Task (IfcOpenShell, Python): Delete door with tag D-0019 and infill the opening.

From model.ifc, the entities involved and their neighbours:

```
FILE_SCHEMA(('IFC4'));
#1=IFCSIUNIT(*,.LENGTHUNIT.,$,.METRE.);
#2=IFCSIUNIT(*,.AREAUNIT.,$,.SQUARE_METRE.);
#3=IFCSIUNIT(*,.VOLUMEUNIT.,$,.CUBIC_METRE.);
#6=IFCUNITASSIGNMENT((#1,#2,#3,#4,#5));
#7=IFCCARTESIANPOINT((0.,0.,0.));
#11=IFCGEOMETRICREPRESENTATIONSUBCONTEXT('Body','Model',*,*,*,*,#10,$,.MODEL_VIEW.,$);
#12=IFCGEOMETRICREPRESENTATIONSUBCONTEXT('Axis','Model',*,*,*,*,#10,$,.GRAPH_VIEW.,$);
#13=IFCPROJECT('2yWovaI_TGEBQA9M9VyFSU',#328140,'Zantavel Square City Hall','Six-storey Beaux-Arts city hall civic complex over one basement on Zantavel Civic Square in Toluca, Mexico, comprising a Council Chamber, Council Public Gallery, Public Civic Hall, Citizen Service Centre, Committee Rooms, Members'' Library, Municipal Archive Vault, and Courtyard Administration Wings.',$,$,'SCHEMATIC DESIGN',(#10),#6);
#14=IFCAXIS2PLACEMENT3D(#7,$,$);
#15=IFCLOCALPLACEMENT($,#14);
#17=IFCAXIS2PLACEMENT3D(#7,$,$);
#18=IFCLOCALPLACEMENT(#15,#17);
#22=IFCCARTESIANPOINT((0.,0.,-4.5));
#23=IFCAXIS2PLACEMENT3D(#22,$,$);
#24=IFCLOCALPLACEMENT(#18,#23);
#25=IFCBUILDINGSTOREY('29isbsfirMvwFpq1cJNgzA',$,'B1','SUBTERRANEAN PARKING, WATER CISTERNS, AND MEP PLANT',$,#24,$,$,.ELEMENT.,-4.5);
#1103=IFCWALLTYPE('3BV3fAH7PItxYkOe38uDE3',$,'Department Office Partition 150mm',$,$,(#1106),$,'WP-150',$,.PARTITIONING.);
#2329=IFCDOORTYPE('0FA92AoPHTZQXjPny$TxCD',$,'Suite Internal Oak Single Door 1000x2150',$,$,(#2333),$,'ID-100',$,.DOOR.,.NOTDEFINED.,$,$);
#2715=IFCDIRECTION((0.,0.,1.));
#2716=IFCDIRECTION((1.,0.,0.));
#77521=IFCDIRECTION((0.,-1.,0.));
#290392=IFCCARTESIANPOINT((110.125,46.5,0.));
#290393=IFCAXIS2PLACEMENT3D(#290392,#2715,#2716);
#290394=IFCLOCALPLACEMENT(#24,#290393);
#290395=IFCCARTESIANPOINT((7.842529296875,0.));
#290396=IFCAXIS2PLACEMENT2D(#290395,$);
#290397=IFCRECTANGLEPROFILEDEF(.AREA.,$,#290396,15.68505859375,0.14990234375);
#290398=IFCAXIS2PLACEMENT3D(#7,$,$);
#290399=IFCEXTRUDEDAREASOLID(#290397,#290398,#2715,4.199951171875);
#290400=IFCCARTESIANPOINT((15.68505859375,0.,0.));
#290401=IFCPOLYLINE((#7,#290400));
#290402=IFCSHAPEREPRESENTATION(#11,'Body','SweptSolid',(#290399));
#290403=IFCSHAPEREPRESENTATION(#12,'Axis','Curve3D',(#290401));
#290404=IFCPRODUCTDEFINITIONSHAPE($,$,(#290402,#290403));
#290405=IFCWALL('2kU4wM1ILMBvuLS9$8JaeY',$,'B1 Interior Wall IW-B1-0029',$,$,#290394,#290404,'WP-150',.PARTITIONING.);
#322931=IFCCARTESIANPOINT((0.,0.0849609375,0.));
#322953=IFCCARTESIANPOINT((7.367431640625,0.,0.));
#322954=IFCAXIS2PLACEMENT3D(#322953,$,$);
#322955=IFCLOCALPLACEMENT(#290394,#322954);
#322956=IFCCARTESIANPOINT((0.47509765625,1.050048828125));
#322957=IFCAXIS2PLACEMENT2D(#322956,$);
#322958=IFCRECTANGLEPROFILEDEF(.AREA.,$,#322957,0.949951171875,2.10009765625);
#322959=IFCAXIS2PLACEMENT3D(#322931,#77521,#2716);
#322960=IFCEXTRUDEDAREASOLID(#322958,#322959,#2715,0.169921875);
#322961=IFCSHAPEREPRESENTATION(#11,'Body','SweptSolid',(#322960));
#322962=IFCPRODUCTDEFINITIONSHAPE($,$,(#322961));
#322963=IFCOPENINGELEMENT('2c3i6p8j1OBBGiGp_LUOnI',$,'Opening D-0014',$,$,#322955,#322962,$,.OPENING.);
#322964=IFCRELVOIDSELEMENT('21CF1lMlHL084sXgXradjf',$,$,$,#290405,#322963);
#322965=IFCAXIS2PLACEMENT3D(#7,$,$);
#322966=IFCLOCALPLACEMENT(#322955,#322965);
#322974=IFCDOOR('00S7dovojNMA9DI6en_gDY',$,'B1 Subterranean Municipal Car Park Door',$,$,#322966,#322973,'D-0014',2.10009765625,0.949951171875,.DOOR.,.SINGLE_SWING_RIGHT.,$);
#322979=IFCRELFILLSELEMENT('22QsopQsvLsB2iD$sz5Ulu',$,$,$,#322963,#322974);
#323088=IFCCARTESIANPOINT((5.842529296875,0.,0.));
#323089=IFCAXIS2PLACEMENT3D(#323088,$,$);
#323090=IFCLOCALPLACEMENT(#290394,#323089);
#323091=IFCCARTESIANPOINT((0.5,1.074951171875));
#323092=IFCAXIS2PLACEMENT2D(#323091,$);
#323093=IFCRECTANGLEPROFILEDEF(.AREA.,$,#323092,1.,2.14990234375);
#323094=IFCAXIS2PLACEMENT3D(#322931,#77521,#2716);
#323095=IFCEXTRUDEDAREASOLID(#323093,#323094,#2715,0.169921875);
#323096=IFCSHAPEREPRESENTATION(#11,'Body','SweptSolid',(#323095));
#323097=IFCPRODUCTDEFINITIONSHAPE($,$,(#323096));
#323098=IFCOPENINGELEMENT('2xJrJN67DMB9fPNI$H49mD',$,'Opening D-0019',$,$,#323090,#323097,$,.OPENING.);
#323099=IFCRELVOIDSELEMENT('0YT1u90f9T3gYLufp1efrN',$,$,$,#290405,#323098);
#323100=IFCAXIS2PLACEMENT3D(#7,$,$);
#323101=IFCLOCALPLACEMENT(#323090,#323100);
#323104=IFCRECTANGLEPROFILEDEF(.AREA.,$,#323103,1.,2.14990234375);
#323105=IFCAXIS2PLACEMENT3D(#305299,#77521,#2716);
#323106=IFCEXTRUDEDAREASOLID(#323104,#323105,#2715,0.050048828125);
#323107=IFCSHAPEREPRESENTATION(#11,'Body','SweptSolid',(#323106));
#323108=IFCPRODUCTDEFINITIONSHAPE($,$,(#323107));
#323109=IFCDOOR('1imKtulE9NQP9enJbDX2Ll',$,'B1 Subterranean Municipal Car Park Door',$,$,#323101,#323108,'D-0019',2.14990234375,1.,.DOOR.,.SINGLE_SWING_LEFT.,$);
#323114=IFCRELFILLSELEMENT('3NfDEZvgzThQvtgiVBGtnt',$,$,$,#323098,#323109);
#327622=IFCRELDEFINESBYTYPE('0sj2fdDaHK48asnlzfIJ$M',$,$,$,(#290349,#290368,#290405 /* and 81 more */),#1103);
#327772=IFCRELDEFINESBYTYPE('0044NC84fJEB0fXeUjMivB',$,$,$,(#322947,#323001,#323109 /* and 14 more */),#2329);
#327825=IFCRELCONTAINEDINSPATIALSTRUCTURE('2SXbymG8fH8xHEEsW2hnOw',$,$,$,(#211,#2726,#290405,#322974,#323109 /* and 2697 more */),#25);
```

```python
import ifcopenshell
import ifcopenshell.api.feature
import ifcopenshell.api.root
import ifcopenshell.geom
import ifcopenshell.util.shape

model = ifcopenshell.open("model.ifc")
settings = ifcopenshell.geom.settings()


def volume(element):
    """Net volume in cubic metres, openings subtracted."""
    shape = ifcopenshell.geom.create_shape(settings, element)
    return ifcopenshell.util.shape.get_volume(shape.geometry)


door = model.by_guid("1imKtulE9NQP9enJbDX2Ll")
opening = door.FillsVoids[0].RelatingOpeningElement
wall = opening.VoidsElements[0].RelatingBuildingElement
before = volume(wall)

ifcopenshell.api.root.remove_product(model, product=door)
ifcopenshell.api.feature.remove_feature(model, feature=opening)

after = volume(wall)

print(f"wall volume {before:.3f} -> {after:.3f} m3")

model.write("model_edited.ifc")
```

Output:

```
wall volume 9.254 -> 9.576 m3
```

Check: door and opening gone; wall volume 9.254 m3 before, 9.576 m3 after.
